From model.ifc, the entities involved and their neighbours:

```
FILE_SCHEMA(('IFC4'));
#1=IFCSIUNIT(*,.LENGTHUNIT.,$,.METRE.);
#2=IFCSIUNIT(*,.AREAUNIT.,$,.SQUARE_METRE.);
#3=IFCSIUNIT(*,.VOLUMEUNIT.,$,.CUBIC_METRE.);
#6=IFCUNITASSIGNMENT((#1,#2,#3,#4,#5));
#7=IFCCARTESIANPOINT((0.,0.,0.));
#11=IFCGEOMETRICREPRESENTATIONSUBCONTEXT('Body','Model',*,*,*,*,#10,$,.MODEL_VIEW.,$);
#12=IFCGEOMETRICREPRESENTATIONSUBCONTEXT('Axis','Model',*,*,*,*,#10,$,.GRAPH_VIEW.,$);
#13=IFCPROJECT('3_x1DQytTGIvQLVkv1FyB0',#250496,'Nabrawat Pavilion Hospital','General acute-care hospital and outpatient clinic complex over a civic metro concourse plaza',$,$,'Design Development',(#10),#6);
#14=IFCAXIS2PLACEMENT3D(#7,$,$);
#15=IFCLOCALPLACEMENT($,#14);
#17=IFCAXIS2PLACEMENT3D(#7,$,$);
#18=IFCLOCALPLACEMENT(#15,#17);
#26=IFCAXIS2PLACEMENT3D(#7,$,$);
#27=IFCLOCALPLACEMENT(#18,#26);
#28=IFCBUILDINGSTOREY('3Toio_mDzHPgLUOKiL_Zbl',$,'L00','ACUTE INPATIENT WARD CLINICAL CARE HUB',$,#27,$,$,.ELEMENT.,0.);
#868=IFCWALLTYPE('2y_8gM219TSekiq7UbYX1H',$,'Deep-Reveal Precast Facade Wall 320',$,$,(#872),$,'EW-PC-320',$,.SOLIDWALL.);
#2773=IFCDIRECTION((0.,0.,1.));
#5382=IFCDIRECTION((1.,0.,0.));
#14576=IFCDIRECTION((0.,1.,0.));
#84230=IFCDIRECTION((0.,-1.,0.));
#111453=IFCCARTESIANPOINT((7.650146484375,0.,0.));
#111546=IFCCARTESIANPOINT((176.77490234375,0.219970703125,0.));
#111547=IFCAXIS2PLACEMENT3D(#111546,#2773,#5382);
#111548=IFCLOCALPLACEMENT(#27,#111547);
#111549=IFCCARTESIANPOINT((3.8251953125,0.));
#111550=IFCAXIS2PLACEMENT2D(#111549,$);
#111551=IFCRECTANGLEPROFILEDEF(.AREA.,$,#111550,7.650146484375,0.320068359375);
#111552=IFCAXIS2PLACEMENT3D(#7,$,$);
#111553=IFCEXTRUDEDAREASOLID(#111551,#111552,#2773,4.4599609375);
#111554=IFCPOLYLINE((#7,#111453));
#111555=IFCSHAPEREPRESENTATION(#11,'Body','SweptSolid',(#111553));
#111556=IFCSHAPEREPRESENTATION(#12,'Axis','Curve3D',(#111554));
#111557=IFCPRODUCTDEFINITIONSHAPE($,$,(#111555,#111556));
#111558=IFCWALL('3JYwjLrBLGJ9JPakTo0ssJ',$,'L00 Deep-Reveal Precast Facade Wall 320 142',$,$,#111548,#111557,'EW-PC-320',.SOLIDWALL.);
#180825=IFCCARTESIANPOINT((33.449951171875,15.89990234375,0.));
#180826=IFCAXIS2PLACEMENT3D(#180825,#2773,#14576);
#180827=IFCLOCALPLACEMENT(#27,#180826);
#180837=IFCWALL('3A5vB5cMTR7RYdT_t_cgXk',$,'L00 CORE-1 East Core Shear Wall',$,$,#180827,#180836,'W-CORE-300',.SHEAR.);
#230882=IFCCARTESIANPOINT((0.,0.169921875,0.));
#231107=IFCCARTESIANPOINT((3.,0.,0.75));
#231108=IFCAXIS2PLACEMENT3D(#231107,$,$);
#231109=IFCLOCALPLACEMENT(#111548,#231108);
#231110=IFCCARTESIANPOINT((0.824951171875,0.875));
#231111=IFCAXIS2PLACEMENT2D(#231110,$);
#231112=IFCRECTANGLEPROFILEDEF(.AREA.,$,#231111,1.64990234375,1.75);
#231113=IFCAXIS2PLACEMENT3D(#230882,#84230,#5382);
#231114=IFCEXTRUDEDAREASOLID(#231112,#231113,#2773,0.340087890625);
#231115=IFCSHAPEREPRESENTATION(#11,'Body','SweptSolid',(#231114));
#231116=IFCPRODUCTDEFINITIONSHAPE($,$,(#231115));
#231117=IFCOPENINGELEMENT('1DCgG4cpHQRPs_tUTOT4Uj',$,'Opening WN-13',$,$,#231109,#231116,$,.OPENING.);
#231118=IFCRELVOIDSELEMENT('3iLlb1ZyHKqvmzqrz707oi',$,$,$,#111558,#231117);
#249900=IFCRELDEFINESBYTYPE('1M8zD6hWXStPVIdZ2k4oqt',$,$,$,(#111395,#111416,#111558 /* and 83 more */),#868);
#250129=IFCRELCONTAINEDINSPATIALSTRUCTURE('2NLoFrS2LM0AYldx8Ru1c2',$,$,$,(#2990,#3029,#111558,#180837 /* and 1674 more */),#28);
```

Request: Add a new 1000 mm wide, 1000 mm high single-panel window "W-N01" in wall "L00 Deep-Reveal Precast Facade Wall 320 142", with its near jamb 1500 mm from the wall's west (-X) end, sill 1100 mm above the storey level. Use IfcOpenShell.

```python
import numpy as np
import ifcopenshell
import ifcopenshell.api.feature
import ifcopenshell.api.geometry
import ifcopenshell.api.root
import ifcopenshell.api.spatial
import ifcopenshell.geom
import ifcopenshell.util.element
import ifcopenshell.util.placement
import ifcopenshell.util.representation
import ifcopenshell.util.shape
import ifcopenshell.util.unit

model = ifcopenshell.open("model.ifc")
unit_scale = ifcopenshell.util.unit.calculate_unit_scale(model)
settings = ifcopenshell.geom.settings()


def volume(element):
    """Net volume in cubic metres, openings subtracted."""
    shape = ifcopenshell.geom.create_shape(settings, element)
    return ifcopenshell.util.shape.get_volume(shape.geometry)


wall = model.by_guid("3JYwjLrBLGJ9JPakTo0ssJ")
storey = ifcopenshell.util.element.get_container(wall, ifc_class="IfcBuildingStorey")
context = ifcopenshell.util.representation.get_context(model, "Model", "Body", "MODEL_VIEW")
before = volume(wall)

width, height, from_end, sill = 1, 1, 1.5, 1.1  # metres

# The wall runs along its own X axis, and the end named is its -X end.
wall_shape = ifcopenshell.geom.create_shape(settings, wall)
x, y, z = ifcopenshell.util.shape.get_vertices(wall_shape.geometry).T
start = x.min() + from_end
face, thickness = float(y.min()), float(y.max() - y.min())
wall_matrix = ifcopenshell.util.placement.get_local_placement(wall.ObjectPlacement)
level = ifcopenshell.util.placement.get_local_placement(storey.ObjectPlacement)[2, 3]


def in_wall(x, y):
    """Placement at x, y metres in the wall's axes, at sill height."""
    matrix = wall_matrix.copy()
    matrix[:, 3] = wall_matrix @ np.array([x / unit_scale, y / unit_scale, 0.0, 1.0])
    matrix[2, 3] = level + sill / unit_scale
    return matrix


# Opening: a box that overshoots both wall faces by 50 mm.
opening = ifcopenshell.api.root.create_entity(model, ifc_class="IfcOpeningElement", predefined_type="OPENING")
box = ifcopenshell.api.geometry.add_wall_representation(
    model, context=context, length=width, height=height, thickness=thickness + 0.1
)
ifcopenshell.api.geometry.assign_representation(model, product=opening, representation=box)
ifcopenshell.api.geometry.edit_object_placement(model, product=opening, matrix=in_wall(start, face - 0.05), is_si=False)
ifcopenshell.api.feature.add_feature(model, feature=opening, element=wall)

window = ifcopenshell.api.root.create_entity(model, ifc_class="IfcWindow", name="W-N01", predefined_type="WINDOW")
window.OverallWidth, window.OverallHeight = width / unit_scale, height / unit_scale
window.PartitioningType = "SINGLE_PANEL"
body = ifcopenshell.api.geometry.add_window_representation(
    model,
    context=context,
    overall_width=window.OverallWidth,
    overall_height=window.OverallHeight,
    partition_type="SINGLE_PANEL",
)
ifcopenshell.api.geometry.assign_representation(model, product=window, representation=body)
ifcopenshell.api.spatial.assign_container(model, products=[window], relating_structure=storey)
ifcopenshell.api.feature.add_filling(model, opening=opening, element=window)

# Centre the window in the wall's thickness.
ifcopenshell.api.geometry.edit_object_placement(model, product=window, matrix=in_wall(start, face), is_si=False)
window_shape = ifcopenshell.geom.create_shape(settings, window)
depth = ifcopenshell.util.shape.get_vertices(window_shape.geometry)[:, 1]
offset = face + thickness / 2 - (depth.min() + depth.max()) / 2
ifcopenshell.api.geometry.edit_object_placement(model, product=window, matrix=in_wall(start, offset), is_si=False)

after = volume(wall)

print(f"wall volume {before:.3f} -> {after:.3f} m3")

model.write("model_edited.ifc")
```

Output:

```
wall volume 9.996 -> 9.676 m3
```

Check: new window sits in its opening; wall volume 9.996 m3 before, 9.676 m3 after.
